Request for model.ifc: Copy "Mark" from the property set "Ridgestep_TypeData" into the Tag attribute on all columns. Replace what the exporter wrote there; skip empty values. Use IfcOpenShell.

First a look at what the model holds.

```python
import ifcopenshell
import ifcopenshell.util.element

model = ifcopenshell.open("model.ifc")
print(model.schema)
columns = model.by_type("IfcColumn")
print(len(columns), "columns")
for e in columns[:8]:
    source = ifcopenshell.util.element.get_pset(e, "Ridgestep_TypeData", "Mark")
    target = e.Tag
    print(e.id(), repr(source), repr(target), sep=" | ")
```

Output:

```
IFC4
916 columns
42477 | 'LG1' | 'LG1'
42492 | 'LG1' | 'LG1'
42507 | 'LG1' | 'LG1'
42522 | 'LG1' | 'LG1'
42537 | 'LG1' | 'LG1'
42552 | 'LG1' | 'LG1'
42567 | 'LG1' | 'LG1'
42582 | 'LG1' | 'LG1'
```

```python
import ifcopenshell
import ifcopenshell.util.element

model = ifcopenshell.open("model.ifc")

count = 0
for e in model.by_type("IfcColumn"):
    value = ifcopenshell.util.element.get_pset(e, "Ridgestep_TypeData", "Mark")
    current = e.Tag
    if not value or not value.strip() or current == value:
        continue
    e.Tag = value
    count += 1

print(count, "columns updated")

model.write("model-out.ifc")
```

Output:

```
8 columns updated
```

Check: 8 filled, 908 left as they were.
